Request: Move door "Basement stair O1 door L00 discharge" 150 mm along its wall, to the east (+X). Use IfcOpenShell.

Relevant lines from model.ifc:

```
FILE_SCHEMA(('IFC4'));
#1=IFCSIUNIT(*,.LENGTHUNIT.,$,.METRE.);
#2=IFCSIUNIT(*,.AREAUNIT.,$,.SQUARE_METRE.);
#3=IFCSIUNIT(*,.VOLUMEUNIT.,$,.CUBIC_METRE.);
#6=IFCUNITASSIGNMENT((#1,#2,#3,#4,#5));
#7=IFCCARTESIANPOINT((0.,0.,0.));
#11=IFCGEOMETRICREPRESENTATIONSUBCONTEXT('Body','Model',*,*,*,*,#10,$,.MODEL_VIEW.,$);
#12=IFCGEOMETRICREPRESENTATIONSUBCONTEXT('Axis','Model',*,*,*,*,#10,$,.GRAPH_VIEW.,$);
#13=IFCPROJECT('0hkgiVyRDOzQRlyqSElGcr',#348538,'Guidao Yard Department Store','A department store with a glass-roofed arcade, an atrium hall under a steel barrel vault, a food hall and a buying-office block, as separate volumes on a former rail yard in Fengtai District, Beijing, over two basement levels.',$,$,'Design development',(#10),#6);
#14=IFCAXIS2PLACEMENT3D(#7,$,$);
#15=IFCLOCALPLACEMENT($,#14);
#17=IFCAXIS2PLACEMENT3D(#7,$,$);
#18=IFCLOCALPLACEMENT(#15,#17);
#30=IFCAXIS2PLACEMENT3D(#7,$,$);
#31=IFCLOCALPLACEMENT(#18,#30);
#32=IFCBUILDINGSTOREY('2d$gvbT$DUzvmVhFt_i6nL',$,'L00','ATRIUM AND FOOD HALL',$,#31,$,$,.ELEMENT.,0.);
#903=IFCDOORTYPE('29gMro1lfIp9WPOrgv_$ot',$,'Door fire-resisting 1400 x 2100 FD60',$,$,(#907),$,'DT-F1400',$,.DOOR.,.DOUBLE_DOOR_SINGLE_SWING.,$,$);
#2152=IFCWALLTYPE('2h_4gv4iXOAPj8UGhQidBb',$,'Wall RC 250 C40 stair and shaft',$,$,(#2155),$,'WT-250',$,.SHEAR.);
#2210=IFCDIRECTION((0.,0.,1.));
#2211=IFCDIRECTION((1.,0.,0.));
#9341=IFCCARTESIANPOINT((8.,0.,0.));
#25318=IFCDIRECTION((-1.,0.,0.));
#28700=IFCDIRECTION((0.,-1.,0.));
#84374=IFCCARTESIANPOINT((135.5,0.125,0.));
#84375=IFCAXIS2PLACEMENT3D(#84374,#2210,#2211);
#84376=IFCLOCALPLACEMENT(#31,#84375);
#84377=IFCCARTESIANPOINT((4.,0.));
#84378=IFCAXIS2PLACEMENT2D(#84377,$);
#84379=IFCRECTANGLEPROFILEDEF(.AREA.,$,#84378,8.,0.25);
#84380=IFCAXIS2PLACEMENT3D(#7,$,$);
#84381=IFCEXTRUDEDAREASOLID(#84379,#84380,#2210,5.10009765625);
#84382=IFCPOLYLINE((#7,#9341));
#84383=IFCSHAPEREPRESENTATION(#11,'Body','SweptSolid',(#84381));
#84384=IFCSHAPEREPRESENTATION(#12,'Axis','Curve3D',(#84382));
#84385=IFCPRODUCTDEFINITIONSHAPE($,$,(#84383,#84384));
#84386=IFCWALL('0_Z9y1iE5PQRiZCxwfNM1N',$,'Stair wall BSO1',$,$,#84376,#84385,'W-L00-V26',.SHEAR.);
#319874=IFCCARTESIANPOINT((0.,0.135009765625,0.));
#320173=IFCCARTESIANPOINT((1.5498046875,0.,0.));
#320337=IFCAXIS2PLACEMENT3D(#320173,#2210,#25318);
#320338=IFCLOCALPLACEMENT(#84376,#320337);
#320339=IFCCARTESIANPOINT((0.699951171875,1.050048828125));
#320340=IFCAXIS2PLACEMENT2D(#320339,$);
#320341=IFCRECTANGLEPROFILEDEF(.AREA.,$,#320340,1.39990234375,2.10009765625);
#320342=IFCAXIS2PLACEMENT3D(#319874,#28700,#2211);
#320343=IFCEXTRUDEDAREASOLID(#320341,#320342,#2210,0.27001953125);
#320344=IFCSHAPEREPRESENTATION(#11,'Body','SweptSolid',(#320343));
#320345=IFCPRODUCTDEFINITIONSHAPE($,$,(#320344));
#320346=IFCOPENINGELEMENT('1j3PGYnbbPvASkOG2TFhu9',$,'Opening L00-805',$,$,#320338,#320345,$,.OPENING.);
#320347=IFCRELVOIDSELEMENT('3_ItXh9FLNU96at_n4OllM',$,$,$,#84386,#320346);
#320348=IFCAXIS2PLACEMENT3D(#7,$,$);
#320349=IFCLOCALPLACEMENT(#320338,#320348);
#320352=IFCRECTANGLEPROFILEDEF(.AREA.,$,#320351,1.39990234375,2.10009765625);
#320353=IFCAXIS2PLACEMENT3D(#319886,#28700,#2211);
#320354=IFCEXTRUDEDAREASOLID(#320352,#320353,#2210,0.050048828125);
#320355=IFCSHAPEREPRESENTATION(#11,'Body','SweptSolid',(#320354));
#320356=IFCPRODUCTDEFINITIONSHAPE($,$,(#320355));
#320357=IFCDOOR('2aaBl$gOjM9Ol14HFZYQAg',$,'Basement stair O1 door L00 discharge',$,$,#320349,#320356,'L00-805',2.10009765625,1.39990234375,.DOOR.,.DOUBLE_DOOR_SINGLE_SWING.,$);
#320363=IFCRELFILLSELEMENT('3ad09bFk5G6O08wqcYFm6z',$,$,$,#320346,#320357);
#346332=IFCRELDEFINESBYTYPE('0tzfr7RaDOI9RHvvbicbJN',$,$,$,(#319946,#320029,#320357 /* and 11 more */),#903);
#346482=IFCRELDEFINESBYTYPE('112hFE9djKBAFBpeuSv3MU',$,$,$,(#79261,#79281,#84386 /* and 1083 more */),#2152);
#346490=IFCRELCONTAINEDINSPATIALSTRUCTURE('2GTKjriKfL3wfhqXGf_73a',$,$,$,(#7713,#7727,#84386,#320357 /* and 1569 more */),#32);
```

```python
import ifcopenshell
import ifcopenshell.api.geometry
import ifcopenshell.util.placement

model = ifcopenshell.open("model.ifc")

door = model.by_guid("2aaBl$gOjM9Ol14HFZYQAg")
opening = door.FillsVoids[0].RelatingOpeningElement
wall = opening.VoidsElements[0].RelatingBuildingElement

wall_matrix = ifcopenshell.util.placement.get_local_placement(wall.ObjectPlacement)
shift = wall_matrix[:3, 0] * 0.15
before = ifcopenshell.util.placement.get_local_placement(door.ObjectPlacement)[:3, 3].copy()

# The door is placed relative to its opening, so it follows when the opening moves.
matrix = ifcopenshell.util.placement.get_local_placement(opening.ObjectPlacement)
matrix[:3, 3] += shift
ifcopenshell.api.geometry.edit_object_placement(
    model, product=opening, matrix=matrix, is_si=False, should_transform_children=True
)

after = ifcopenshell.util.placement.get_local_placement(door.ObjectPlacement)[:3, 3]
print("door moved by", (after - before).round(3) + 0.0)

model.write("model_updated.ifc")
```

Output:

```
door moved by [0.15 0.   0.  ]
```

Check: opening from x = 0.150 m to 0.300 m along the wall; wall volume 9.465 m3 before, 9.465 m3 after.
